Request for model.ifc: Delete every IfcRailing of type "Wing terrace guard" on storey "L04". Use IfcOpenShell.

First a look at what the model holds.

```python
import ifcopenshell
import ifcopenshell.util.element

model = ifcopenshell.open("model.ifc")
print(model.schema)
storey = next(s for s in model.by_type("IfcBuildingStorey") if s.Name == "L04")
railings = [e for e in ifcopenshell.util.element.get_decomposition(storey) if e.is_a("IfcRailing")]
seen = {}
for e in railings:
    element_type = ifcopenshell.util.element.get_type(e)
    name = element_type.Name if element_type not in (None, e) else None
    seen[name] = seen.get(name, 0) + 1
for name, count in sorted(seen.items(), key=str):
    print(count, "x", name)
```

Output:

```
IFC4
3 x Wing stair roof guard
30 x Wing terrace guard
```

```python
import ifcopenshell
import ifcopenshell.api.root
import ifcopenshell.util.element

model = ifcopenshell.open("model.ifc")

storey = next(s for s in model.by_type("IfcBuildingStorey") if s.Name == "L04")
railings = [e for e in ifcopenshell.util.element.get_decomposition(storey) if e.is_a("IfcRailing")]
targets = [e for e in railings if (t := ifcopenshell.util.element.get_type(e)) not in (None, e) and t.Name == "Wing terrace guard"]

for e in targets:
    ifcopenshell.api.root.remove_product(model, product=e)
print(len(targets), "removed")

model.write("model_v2.ifc")
```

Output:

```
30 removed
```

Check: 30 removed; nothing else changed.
